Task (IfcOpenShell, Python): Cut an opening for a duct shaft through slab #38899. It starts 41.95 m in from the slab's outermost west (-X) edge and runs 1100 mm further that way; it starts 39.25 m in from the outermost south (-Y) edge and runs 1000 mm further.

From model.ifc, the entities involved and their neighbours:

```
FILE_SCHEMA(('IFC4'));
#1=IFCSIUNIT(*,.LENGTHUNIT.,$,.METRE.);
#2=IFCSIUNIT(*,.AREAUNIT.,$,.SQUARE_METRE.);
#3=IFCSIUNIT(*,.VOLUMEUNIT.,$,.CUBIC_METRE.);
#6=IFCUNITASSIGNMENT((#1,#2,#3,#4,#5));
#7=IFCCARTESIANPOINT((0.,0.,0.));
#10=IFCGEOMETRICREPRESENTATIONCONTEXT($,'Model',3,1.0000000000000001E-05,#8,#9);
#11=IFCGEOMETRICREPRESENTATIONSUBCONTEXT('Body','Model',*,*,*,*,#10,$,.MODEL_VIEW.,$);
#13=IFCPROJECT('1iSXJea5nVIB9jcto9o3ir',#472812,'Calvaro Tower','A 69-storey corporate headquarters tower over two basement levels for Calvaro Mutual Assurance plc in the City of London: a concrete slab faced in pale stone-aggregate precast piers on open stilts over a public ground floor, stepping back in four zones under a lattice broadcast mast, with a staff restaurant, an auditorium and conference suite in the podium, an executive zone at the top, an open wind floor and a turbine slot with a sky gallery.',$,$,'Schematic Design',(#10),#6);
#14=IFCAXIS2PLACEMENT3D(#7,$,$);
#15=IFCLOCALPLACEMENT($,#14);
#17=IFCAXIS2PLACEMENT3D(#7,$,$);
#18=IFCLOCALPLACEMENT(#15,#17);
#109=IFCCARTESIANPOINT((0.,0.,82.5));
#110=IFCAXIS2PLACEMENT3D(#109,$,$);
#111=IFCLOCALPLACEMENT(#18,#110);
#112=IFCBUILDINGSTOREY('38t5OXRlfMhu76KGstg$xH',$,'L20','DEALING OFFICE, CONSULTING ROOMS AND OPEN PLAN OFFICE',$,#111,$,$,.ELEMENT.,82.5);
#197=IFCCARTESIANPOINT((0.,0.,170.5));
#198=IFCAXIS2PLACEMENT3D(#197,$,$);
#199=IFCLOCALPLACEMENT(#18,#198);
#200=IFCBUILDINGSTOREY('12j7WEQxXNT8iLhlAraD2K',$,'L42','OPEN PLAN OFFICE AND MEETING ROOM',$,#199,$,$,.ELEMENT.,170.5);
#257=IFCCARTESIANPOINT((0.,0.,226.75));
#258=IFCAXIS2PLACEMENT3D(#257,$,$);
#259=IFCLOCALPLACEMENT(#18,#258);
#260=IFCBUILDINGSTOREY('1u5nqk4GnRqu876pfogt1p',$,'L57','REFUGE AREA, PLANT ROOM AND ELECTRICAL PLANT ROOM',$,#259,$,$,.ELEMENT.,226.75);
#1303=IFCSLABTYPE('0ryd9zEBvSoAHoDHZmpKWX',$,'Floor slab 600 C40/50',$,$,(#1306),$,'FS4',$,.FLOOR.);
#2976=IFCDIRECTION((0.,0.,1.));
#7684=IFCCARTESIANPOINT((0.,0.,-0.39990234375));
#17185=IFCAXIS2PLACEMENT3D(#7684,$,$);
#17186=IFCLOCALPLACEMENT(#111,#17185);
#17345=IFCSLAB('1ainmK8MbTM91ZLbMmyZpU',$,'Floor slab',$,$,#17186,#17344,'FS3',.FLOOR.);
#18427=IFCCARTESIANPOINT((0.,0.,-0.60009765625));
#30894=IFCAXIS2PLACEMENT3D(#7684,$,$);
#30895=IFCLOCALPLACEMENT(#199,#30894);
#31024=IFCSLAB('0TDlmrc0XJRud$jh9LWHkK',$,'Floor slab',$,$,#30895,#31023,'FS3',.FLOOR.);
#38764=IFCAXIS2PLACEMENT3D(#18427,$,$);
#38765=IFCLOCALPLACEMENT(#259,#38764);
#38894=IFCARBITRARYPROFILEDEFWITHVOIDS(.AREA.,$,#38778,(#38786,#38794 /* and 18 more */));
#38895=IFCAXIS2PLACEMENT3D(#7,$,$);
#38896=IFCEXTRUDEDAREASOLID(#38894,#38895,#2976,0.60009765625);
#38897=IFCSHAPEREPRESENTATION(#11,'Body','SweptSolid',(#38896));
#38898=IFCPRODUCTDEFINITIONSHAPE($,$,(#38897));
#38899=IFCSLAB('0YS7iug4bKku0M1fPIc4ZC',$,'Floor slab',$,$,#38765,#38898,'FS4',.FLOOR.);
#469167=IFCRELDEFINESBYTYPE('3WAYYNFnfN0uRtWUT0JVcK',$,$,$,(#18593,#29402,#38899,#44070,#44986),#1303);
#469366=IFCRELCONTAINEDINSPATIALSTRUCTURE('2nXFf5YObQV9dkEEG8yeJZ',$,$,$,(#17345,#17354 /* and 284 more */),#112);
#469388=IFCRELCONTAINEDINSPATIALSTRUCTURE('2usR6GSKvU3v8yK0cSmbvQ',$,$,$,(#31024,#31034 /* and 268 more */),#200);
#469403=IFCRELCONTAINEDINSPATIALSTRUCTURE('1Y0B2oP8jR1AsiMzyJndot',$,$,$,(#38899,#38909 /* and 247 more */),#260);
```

```python
import numpy as np
import ifcopenshell
import ifcopenshell.api.feature
import ifcopenshell.api.geometry
import ifcopenshell.api.root
import ifcopenshell.geom
import ifcopenshell.util.placement
import ifcopenshell.util.representation
import ifcopenshell.util.shape
import ifcopenshell.util.unit

model = ifcopenshell.open("model.ifc")
unit_scale = ifcopenshell.util.unit.calculate_unit_scale(model)
settings = ifcopenshell.geom.settings()


def volume(element):
    """Net volume in cubic metres, openings subtracted."""
    shape = ifcopenshell.geom.create_shape(settings, element)
    return ifcopenshell.util.shape.get_volume(shape.geometry)


slab = model.by_id(38899)
before = volume(slab)

# Extent in the slab's own axes, in metres. The edges named are its -X and -Y sides.
slab_shape = ifcopenshell.geom.create_shape(settings, slab)
vertices = ifcopenshell.util.shape.get_vertices(slab_shape.geometry)
x_min, y_min, bottom = vertices.min(axis=0)
top = vertices[:, 2].max()

opening = ifcopenshell.api.root.create_entity(model, ifc_class="IfcOpeningElement", name="Duct shaft opening", predefined_type="OPENING")
context = ifcopenshell.util.representation.get_context(model, "Model", "Body", "MODEL_VIEW")
width, depth = 1.1, 1
outline = [(0.0, 0.0), (width, 0.0), (width, depth), (0.0, depth), (0.0, 0.0)]
# Overshoot both faces by 50 mm so the cut is clean.
shape = ifcopenshell.api.geometry.add_slab_representation(
    model, context=context, depth=top - bottom + 0.1, polyline=outline
)
ifcopenshell.api.geometry.assign_representation(model, product=opening, representation=shape)

matrix = ifcopenshell.util.placement.get_local_placement(slab.ObjectPlacement)
matrix[:, 3] = matrix @ np.append(np.array([x_min + 41.95, y_min + 39.25, bottom - 0.05]) / unit_scale, 1.0)
ifcopenshell.api.geometry.edit_object_placement(model, product=opening, matrix=matrix, is_si=False)
ifcopenshell.api.feature.add_feature(model, feature=opening, element=slab)

after = volume(slab)

print(f"slab volume {before:.3f} -> {after:.3f} m3")

model.write("model-out.ifc")
```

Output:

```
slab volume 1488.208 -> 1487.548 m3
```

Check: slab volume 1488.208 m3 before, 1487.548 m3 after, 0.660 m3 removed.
